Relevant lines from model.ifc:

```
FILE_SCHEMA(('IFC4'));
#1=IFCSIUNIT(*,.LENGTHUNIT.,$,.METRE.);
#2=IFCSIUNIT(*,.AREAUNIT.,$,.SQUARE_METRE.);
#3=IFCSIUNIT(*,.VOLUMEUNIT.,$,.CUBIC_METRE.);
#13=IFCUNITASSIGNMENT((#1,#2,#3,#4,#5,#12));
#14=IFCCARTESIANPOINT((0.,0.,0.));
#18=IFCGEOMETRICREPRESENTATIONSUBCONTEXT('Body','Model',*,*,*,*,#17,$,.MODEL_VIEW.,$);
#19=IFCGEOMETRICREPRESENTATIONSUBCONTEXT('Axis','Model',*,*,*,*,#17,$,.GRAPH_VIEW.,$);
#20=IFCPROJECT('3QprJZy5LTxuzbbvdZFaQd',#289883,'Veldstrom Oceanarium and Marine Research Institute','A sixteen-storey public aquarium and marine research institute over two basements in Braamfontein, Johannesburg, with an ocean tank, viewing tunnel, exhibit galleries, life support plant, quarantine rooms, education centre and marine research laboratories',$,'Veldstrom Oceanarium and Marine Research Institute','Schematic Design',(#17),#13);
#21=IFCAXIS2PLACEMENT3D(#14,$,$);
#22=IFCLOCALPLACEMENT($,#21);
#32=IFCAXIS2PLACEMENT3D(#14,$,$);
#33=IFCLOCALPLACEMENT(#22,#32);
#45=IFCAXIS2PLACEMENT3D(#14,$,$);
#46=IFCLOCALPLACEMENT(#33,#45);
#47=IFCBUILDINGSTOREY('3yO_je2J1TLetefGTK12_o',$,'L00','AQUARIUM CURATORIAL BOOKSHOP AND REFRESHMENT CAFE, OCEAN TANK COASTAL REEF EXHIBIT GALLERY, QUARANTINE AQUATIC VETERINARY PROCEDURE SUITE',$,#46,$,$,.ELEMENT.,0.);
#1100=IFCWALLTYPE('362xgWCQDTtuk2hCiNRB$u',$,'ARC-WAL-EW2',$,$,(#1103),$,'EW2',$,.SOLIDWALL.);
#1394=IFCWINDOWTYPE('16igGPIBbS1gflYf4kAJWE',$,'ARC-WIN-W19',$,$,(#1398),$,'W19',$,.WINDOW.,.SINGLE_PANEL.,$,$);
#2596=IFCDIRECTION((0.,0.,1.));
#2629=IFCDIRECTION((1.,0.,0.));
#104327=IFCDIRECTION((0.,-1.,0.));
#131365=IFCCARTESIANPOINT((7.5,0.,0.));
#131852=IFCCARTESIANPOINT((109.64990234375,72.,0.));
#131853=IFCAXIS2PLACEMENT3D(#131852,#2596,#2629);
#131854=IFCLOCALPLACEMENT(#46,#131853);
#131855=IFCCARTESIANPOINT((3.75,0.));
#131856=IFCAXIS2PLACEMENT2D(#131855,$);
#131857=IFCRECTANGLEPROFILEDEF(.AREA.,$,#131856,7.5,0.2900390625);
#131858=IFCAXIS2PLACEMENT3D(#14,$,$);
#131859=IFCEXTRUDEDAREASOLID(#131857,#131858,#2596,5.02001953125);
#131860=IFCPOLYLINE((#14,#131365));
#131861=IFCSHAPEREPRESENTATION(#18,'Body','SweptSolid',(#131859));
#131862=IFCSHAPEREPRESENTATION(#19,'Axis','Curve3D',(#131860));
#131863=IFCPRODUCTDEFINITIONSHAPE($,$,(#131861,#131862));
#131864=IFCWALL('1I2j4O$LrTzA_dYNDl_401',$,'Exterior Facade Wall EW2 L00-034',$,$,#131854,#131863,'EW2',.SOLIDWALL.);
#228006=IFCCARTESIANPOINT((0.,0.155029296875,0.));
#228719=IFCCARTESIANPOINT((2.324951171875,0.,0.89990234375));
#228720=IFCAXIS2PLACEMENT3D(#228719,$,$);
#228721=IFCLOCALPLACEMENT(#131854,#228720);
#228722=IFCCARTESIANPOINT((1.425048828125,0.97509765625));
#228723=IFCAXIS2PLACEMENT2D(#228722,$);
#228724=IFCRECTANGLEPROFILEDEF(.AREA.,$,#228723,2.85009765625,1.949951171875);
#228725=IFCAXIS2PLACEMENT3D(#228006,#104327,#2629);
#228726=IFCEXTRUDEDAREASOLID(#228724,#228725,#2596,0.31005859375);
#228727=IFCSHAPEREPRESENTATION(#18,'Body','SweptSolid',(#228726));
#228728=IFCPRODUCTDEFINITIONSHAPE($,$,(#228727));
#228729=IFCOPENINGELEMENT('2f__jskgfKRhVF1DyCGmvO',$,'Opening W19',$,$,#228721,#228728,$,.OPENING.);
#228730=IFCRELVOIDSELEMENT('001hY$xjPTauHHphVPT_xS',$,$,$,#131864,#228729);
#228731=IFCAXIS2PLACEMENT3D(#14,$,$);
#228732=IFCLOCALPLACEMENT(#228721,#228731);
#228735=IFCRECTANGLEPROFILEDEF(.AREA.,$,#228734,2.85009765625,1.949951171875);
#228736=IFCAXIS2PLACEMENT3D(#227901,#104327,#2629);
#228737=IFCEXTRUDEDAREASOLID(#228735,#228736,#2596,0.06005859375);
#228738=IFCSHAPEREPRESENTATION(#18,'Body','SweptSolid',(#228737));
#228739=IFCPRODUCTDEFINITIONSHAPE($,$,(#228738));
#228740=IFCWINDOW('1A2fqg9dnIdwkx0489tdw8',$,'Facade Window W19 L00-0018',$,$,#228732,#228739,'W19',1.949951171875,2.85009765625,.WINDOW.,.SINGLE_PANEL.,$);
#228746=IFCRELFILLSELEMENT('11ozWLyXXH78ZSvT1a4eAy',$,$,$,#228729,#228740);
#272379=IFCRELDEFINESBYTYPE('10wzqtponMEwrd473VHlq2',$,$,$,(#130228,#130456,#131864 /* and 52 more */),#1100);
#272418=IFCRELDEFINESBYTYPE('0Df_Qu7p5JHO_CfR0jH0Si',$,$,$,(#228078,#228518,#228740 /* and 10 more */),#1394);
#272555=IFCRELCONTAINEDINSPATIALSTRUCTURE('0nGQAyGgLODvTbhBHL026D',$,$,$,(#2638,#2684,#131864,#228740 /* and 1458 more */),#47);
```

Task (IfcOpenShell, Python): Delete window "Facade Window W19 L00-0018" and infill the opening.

```python
import ifcopenshell
import ifcopenshell.api.feature
import ifcopenshell.api.root
import ifcopenshell.geom
import ifcopenshell.util.shape

model = ifcopenshell.open("model.ifc")
settings = ifcopenshell.geom.settings()


def volume(element):
    """Net volume in cubic metres, openings subtracted."""
    shape = ifcopenshell.geom.create_shape(settings, element)
    return ifcopenshell.util.shape.get_volume(shape.geometry)


window = model.by_id(228740)
opening = window.FillsVoids[0].RelatingOpeningElement
wall = opening.VoidsElements[0].RelatingBuildingElement
before = volume(wall)

ifcopenshell.api.root.remove_product(model, product=window)
ifcopenshell.api.feature.remove_feature(model, feature=opening)

after = volume(wall)

print(f"wall volume {before:.3f} -> {after:.3f} m3")

model.write("model_edited.ifc")
```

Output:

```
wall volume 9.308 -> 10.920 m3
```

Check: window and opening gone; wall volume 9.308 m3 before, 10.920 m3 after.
